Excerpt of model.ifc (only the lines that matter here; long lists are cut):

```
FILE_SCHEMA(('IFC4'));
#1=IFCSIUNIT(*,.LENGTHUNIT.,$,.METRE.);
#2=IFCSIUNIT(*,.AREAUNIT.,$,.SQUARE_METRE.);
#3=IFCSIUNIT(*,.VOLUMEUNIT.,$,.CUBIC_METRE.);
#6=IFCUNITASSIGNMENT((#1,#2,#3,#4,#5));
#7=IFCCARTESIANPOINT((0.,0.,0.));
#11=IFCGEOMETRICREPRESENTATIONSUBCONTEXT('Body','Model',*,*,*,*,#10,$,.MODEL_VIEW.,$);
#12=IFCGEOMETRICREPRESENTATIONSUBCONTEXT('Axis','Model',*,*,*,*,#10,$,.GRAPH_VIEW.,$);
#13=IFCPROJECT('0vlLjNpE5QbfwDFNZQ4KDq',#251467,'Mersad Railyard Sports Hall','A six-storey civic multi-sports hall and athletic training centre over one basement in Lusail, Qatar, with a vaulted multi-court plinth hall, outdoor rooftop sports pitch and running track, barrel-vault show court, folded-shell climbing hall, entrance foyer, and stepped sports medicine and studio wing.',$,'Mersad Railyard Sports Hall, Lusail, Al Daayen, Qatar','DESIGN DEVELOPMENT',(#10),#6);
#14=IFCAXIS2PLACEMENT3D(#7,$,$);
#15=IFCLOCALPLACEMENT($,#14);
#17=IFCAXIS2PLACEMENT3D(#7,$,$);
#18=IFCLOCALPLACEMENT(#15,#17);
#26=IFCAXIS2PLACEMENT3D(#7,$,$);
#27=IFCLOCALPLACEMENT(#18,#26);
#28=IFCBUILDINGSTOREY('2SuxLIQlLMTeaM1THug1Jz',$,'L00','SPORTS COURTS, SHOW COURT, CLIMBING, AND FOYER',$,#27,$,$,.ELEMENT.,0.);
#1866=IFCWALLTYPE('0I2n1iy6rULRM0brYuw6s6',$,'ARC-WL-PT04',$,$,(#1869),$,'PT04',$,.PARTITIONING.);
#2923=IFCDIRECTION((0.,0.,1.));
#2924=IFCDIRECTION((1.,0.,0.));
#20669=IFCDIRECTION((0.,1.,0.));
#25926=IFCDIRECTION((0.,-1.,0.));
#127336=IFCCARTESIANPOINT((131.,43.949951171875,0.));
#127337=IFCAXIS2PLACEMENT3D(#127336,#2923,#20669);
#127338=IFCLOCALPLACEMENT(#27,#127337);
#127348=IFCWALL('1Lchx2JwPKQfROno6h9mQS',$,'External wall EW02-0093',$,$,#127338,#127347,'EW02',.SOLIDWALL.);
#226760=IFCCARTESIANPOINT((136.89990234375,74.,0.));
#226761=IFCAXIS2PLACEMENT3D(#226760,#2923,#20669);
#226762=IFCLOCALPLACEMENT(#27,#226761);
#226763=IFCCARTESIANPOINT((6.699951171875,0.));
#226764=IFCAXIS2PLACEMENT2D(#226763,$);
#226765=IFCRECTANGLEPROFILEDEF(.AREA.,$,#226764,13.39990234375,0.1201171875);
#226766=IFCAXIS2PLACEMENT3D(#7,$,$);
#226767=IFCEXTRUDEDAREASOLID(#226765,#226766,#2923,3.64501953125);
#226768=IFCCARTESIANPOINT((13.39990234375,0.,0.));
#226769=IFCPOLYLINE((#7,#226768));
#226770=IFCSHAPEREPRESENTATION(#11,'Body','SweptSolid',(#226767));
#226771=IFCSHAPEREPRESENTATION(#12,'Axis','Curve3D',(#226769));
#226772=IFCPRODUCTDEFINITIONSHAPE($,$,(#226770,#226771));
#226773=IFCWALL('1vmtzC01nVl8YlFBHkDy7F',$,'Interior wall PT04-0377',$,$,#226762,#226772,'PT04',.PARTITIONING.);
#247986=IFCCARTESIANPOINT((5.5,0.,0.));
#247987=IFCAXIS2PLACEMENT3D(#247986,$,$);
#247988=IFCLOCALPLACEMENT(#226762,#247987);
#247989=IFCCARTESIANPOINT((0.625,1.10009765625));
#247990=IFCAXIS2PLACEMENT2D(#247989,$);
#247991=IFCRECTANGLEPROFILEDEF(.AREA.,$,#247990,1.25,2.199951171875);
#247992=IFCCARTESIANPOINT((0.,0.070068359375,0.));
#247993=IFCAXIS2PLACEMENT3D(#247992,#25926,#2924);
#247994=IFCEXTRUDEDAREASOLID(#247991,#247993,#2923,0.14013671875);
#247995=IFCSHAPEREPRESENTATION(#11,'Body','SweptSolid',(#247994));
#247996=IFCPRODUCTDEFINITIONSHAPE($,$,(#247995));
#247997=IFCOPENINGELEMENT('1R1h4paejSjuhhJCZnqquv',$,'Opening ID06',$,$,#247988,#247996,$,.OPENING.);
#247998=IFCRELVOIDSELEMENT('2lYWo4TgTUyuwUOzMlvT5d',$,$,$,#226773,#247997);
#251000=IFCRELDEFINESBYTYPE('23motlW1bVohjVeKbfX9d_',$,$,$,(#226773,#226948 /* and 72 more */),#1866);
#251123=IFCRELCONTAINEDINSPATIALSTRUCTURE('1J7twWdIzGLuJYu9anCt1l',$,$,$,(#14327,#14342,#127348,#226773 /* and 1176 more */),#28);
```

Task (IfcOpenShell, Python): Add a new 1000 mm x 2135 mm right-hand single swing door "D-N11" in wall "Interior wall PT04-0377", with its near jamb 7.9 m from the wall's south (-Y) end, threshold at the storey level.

```python
import numpy as np
import ifcopenshell
import ifcopenshell.api.feature
import ifcopenshell.api.geometry
import ifcopenshell.api.root
import ifcopenshell.api.spatial
import ifcopenshell.geom
import ifcopenshell.util.element
import ifcopenshell.util.placement
import ifcopenshell.util.representation
import ifcopenshell.util.shape
import ifcopenshell.util.unit

model = ifcopenshell.open("model.ifc")
unit_scale = ifcopenshell.util.unit.calculate_unit_scale(model)
settings = ifcopenshell.geom.settings()


def volume(element):
    """Net volume in cubic metres, openings subtracted."""
    shape = ifcopenshell.geom.create_shape(settings, element)
    return ifcopenshell.util.shape.get_volume(shape.geometry)


wall = model.by_guid("1vmtzC01nVl8YlFBHkDy7F")
storey = ifcopenshell.util.element.get_container(wall, ifc_class="IfcBuildingStorey")
context = ifcopenshell.util.representation.get_context(model, "Model", "Body", "MODEL_VIEW")
before = volume(wall)

width, height, from_end, sill = 1, 2.135, 7.9, 0.0  # metres

# The wall runs along its own X axis, and the end named is its -X end.
wall_shape = ifcopenshell.geom.create_shape(settings, wall)
x, y, z = ifcopenshell.util.shape.get_vertices(wall_shape.geometry).T
start = x.min() + from_end
face, thickness = float(y.min()), float(y.max() - y.min())
wall_matrix = ifcopenshell.util.placement.get_local_placement(wall.ObjectPlacement)
level = ifcopenshell.util.placement.get_local_placement(storey.ObjectPlacement)[2, 3]


def in_wall(x, y):
    """Placement at x, y metres in the wall's axes, at sill height."""
    matrix = wall_matrix.copy()
    matrix[:, 3] = wall_matrix @ np.array([x / unit_scale, y / unit_scale, 0.0, 1.0])
    matrix[2, 3] = level + sill / unit_scale
    return matrix


# Opening: a box that overshoots both wall faces by 50 mm.
opening = ifcopenshell.api.root.create_entity(model, ifc_class="IfcOpeningElement", predefined_type="OPENING")
box = ifcopenshell.api.geometry.add_wall_representation(
    model, context=context, length=width, height=height, thickness=thickness + 0.1
)
ifcopenshell.api.geometry.assign_representation(model, product=opening, representation=box)
ifcopenshell.api.geometry.edit_object_placement(model, product=opening, matrix=in_wall(start, face - 0.05), is_si=False)
ifcopenshell.api.feature.add_feature(model, feature=opening, element=wall)

door = ifcopenshell.api.root.create_entity(model, ifc_class="IfcDoor", name="D-N11", predefined_type="DOOR")
door.OverallWidth, door.OverallHeight = width / unit_scale, height / unit_scale
door.OperationType = "SINGLE_SWING_RIGHT"
body = ifcopenshell.api.geometry.add_door_representation(
    model,
    context=context,
    overall_width=door.OverallWidth,
    overall_height=door.OverallHeight,
    operation_type="SINGLE_SWING_RIGHT",
    lining_properties={"LiningDepth": thickness / unit_scale, "ThresholdDepth": thickness / unit_scale},
)
ifcopenshell.api.geometry.assign_representation(model, product=door, representation=body)
ifcopenshell.api.spatial.assign_container(model, products=[door], relating_structure=storey)
ifcopenshell.api.feature.add_filling(model, opening=opening, element=door)

# The lining spans the wall, so the door starts at the wall face.
ifcopenshell.api.geometry.edit_object_placement(model, product=door, matrix=in_wall(start, face), is_si=False)

after = volume(wall)

print(f"wall volume {before:.3f} -> {after:.3f} m3")

model.write("model_edited.ifc")
```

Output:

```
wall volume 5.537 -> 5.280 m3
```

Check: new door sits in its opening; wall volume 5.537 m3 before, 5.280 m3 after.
